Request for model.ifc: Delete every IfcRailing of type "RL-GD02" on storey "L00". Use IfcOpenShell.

First a look at what the model holds.

```python
import ifcopenshell
import ifcopenshell.util.element

model = ifcopenshell.open("model.ifc")
print(model.schema)
storey = next(s for s in model.by_type("IfcBuildingStorey") if s.Name == "L00")
railings = [e for e in ifcopenshell.util.element.get_decomposition(storey) if e.is_a("IfcRailing")]
seen = {}
for e in railings:
    element_type = ifcopenshell.util.element.get_type(e)
    name = element_type.Name if element_type not in (None, e) else None
    seen[name] = seen.get(name, 0) + 1
for name, count in sorted(seen.items(), key=str):
    print(count, "x", name)
```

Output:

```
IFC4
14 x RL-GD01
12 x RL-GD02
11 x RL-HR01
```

```python
import ifcopenshell
import ifcopenshell.api.root
import ifcopenshell.util.element

model = ifcopenshell.open("model.ifc")

storey = next(s for s in model.by_type("IfcBuildingStorey") if s.Name == "L00")
railings = [e for e in ifcopenshell.util.element.get_decomposition(storey) if e.is_a("IfcRailing")]
targets = [e for e in railings if (t := ifcopenshell.util.element.get_type(e)) not in (None, e) and t.Name == "RL-GD02"]

for e in targets:
    ifcopenshell.api.root.remove_product(model, product=e)
print(len(targets), "removed")

model.write("model_edited.ifc")
```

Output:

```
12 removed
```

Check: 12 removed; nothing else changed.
